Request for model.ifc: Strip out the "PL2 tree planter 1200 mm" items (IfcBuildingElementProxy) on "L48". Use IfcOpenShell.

First a look at what the model holds.

```python
import ifcopenshell
import ifcopenshell.util.element

model = ifcopenshell.open("model.ifc")
print(model.schema)
storey = next(s for s in model.by_type("IfcBuildingStorey") if s.Name == "L48")
proxies = [e for e in ifcopenshell.util.element.get_decomposition(storey) if e.is_a("IfcBuildingElementProxy")]
seen = {}
for e in proxies:
    element_type = ifcopenshell.util.element.get_type(e)
    name = element_type.Name if element_type not in (None, e) else None
    seen[name] = seen.get(name, 0) + 1
for name, count in sorted(seen.items(), key=str):
    print(count, "x", name)
```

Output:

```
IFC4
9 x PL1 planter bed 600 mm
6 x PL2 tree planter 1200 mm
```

```python
import ifcopenshell
import ifcopenshell.api.root
import ifcopenshell.util.element

model = ifcopenshell.open("model.ifc")

storey = next(s for s in model.by_type("IfcBuildingStorey") if s.Name == "L48")
proxies = [e for e in ifcopenshell.util.element.get_decomposition(storey) if e.is_a("IfcBuildingElementProxy")]
targets = [e for e in proxies if (t := ifcopenshell.util.element.get_type(e)) not in (None, e) and t.Name == "PL2 tree planter 1200 mm"]

for e in targets:
    ifcopenshell.api.root.remove_product(model, product=e)
print(len(targets), "removed")

model.write("model_updated.ifc")
```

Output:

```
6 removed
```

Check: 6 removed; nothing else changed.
